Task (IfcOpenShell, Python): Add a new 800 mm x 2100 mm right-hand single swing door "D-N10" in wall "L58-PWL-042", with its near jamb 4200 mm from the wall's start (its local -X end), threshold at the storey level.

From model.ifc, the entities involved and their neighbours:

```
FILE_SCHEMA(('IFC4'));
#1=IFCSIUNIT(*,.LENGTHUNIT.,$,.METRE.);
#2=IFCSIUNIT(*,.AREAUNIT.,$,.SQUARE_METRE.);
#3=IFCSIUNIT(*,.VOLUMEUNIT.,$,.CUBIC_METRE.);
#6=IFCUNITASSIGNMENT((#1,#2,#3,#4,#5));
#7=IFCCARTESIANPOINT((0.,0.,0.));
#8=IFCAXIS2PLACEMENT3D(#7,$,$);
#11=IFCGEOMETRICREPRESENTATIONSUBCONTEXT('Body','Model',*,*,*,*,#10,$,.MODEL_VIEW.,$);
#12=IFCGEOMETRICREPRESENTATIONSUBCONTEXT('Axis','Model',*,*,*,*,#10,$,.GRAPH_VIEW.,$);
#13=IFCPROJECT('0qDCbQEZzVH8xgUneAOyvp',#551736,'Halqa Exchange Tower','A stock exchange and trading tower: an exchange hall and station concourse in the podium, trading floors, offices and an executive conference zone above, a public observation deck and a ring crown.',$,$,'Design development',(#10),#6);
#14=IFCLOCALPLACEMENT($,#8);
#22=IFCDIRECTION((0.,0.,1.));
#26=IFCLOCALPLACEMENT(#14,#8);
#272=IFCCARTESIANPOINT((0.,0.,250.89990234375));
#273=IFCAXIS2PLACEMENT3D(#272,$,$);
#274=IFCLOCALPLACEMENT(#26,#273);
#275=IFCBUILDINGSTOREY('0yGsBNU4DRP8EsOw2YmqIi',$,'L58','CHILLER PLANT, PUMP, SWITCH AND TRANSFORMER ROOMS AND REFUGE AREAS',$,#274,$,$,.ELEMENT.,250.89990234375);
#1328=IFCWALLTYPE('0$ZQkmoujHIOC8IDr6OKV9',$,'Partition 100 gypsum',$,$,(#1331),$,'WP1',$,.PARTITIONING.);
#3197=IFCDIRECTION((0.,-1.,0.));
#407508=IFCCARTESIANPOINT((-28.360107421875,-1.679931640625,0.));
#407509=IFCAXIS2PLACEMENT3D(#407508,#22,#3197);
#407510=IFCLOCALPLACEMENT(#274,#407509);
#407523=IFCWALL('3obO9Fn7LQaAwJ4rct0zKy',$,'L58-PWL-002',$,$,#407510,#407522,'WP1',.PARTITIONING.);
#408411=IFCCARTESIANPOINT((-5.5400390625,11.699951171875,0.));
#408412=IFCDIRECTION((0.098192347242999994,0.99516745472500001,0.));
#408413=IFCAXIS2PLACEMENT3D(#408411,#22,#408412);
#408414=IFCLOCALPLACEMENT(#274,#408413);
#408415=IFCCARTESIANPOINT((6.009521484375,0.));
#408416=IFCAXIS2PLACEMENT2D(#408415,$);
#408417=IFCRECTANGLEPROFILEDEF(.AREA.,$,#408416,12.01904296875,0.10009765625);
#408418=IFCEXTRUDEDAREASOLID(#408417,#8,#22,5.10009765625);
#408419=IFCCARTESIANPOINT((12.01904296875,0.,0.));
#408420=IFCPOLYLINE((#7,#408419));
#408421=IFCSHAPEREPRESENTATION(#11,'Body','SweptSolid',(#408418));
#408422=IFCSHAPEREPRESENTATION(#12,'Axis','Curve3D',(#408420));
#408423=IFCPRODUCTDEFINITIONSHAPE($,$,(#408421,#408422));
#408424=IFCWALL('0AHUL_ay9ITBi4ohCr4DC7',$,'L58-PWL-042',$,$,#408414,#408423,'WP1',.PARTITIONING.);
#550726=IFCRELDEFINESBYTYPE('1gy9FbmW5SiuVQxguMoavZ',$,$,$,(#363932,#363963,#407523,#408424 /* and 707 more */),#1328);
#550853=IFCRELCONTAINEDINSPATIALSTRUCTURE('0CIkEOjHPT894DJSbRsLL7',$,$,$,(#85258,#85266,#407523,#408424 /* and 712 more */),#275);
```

```python
import numpy as np
import ifcopenshell
import ifcopenshell.api.feature
import ifcopenshell.api.geometry
import ifcopenshell.api.root
import ifcopenshell.api.spatial
import ifcopenshell.geom
import ifcopenshell.util.element
import ifcopenshell.util.placement
import ifcopenshell.util.representation
import ifcopenshell.util.shape
import ifcopenshell.util.unit

model = ifcopenshell.open("model.ifc")
unit_scale = ifcopenshell.util.unit.calculate_unit_scale(model)
settings = ifcopenshell.geom.settings()


def volume(element):
    """Net volume in cubic metres, openings subtracted."""
    shape = ifcopenshell.geom.create_shape(settings, element)
    return ifcopenshell.util.shape.get_volume(shape.geometry)


wall = model.by_guid("0AHUL_ay9ITBi4ohCr4DC7")
storey = ifcopenshell.util.element.get_container(wall, ifc_class="IfcBuildingStorey")
context = ifcopenshell.util.representation.get_context(model, "Model", "Body", "MODEL_VIEW")
before = volume(wall)

width, height, from_end, sill = 0.8, 2.1, 4.2, 0.0  # metres

# The wall runs along its own X axis, and the end named is its -X end.
wall_shape = ifcopenshell.geom.create_shape(settings, wall)
x, y, z = ifcopenshell.util.shape.get_vertices(wall_shape.geometry).T
start = x.min() + from_end
face, thickness = float(y.min()), float(y.max() - y.min())
wall_matrix = ifcopenshell.util.placement.get_local_placement(wall.ObjectPlacement)
level = ifcopenshell.util.placement.get_local_placement(storey.ObjectPlacement)[2, 3]


def in_wall(x, y):
    """Placement at x, y metres in the wall's axes, at sill height."""
    matrix = wall_matrix.copy()
    matrix[:, 3] = wall_matrix @ np.array([x / unit_scale, y / unit_scale, 0.0, 1.0])
    matrix[2, 3] = level + sill / unit_scale
    return matrix


# Opening: a box that overshoots both wall faces by 50 mm.
opening = ifcopenshell.api.root.create_entity(model, ifc_class="IfcOpeningElement", predefined_type="OPENING")
box = ifcopenshell.api.geometry.add_wall_representation(
    model, context=context, length=width, height=height, thickness=thickness + 0.1
)
ifcopenshell.api.geometry.assign_representation(model, product=opening, representation=box)
ifcopenshell.api.geometry.edit_object_placement(model, product=opening, matrix=in_wall(start, face - 0.05), is_si=False)
ifcopenshell.api.feature.add_feature(model, feature=opening, element=wall)

door = ifcopenshell.api.root.create_entity(model, ifc_class="IfcDoor", name="D-N10", predefined_type="DOOR")
door.OverallWidth, door.OverallHeight = width / unit_scale, height / unit_scale
door.OperationType = "SINGLE_SWING_RIGHT"
body = ifcopenshell.api.geometry.add_door_representation(
    model,
    context=context,
    overall_width=door.OverallWidth,
    overall_height=door.OverallHeight,
    operation_type="SINGLE_SWING_RIGHT",
    lining_properties={"LiningDepth": thickness / unit_scale, "ThresholdDepth": thickness / unit_scale},
)
ifcopenshell.api.geometry.assign_representation(model, product=door, representation=body)
ifcopenshell.api.spatial.assign_container(model, products=[door], relating_structure=storey)
ifcopenshell.api.feature.add_filling(model, opening=opening, element=door)

# The lining spans the wall, so the door starts at the wall face.
ifcopenshell.api.geometry.edit_object_placement(model, product=door, matrix=in_wall(start, face), is_si=False)

after = volume(wall)

print(f"wall volume {before:.3f} -> {after:.3f} m3")

model.write("model_updated.ifc")
```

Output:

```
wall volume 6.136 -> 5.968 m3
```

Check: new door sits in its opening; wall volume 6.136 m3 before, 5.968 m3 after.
